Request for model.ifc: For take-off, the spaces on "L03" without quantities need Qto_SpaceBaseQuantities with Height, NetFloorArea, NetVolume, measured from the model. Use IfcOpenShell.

First a look at what the model holds.

```python
import ifcopenshell
import ifcopenshell.util.element
import ifcopenshell.util.unit

model = ifcopenshell.open("model.ifc")
print(model.schema)
for unit_type in ("LENGTHUNIT", "AREAUNIT", "VOLUMEUNIT"):
    print(unit_type, ifcopenshell.util.unit.calculate_unit_scale(model, unit_type))
storey = next(s for s in model.by_type("IfcBuildingStorey") if s.Name == "L03")
spaces = [e for e in ifcopenshell.util.element.get_decomposition(storey) if e.is_a("IfcSpace")]
for e in sorted(spaces, key=lambda e: e.id()):
    print(e.id(), e.is_a(), e.Name, list(ifcopenshell.util.element.get_psets(e, qtos_only=True)), sep=" | ")
```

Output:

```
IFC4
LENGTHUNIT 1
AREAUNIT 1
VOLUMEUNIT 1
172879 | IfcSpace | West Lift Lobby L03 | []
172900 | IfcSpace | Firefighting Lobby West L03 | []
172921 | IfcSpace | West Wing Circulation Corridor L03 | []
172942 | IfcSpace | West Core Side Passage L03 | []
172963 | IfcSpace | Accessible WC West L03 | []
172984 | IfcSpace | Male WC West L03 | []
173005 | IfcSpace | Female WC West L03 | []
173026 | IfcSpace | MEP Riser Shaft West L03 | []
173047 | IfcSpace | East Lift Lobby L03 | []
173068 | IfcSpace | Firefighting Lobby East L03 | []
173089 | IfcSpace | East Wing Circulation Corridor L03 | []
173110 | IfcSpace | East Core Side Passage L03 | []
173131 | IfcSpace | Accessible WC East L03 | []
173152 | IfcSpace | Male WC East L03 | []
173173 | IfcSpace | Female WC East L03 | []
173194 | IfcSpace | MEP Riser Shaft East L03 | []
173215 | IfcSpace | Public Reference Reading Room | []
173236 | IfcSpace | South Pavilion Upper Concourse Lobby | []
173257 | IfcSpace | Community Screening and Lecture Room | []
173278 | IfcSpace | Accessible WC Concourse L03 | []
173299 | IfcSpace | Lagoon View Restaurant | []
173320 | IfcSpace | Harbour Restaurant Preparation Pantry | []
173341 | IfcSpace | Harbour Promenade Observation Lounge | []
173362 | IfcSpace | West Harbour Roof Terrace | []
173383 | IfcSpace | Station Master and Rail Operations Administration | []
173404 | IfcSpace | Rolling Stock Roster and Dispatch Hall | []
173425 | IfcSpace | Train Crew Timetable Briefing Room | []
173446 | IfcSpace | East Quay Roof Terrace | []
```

```python
import ifcopenshell
import ifcopenshell.api.pset
import ifcopenshell.geom
import ifcopenshell.util.element
import ifcopenshell.util.shape
import ifcopenshell.util.unit

model = ifcopenshell.open("model.ifc")
unit_scale = ifcopenshell.util.unit.calculate_unit_scale(model)
area_scale = ifcopenshell.util.unit.calculate_unit_scale(model, "AREAUNIT")
volume_scale = ifcopenshell.util.unit.calculate_unit_scale(model, "VOLUMEUNIT")
settings = ifcopenshell.geom.settings()

storey = next(s for s in model.by_type("IfcBuildingStorey") if s.Name == "L03")
spaces = [e for e in ifcopenshell.util.element.get_decomposition(storey) if e.is_a("IfcSpace")]

for e in sorted(spaces, key=lambda e: e.id()):
    if ifcopenshell.util.element.get_psets(e, qtos_only=True, should_inherit=False):
        continue
    # Geometry comes back in metres, in the element's own axes.
    shape = ifcopenshell.geom.create_shape(settings, e)
    values = {
        "Height": ifcopenshell.util.shape.get_z(shape.geometry) / unit_scale,
        "NetFloorArea": ifcopenshell.util.shape.get_footprint_area(shape.geometry) / area_scale,
        "NetVolume": ifcopenshell.util.shape.get_volume(shape.geometry) / volume_scale,
    }
    qto = ifcopenshell.api.pset.add_qto(model, product=e, name="Qto_SpaceBaseQuantities")
    ifcopenshell.api.pset.edit_qto(model, qto=qto, properties=values)
    print(e.id(), {k: round(v, 3) for k, v in values.items()})

model.write("model_edited.ifc")
```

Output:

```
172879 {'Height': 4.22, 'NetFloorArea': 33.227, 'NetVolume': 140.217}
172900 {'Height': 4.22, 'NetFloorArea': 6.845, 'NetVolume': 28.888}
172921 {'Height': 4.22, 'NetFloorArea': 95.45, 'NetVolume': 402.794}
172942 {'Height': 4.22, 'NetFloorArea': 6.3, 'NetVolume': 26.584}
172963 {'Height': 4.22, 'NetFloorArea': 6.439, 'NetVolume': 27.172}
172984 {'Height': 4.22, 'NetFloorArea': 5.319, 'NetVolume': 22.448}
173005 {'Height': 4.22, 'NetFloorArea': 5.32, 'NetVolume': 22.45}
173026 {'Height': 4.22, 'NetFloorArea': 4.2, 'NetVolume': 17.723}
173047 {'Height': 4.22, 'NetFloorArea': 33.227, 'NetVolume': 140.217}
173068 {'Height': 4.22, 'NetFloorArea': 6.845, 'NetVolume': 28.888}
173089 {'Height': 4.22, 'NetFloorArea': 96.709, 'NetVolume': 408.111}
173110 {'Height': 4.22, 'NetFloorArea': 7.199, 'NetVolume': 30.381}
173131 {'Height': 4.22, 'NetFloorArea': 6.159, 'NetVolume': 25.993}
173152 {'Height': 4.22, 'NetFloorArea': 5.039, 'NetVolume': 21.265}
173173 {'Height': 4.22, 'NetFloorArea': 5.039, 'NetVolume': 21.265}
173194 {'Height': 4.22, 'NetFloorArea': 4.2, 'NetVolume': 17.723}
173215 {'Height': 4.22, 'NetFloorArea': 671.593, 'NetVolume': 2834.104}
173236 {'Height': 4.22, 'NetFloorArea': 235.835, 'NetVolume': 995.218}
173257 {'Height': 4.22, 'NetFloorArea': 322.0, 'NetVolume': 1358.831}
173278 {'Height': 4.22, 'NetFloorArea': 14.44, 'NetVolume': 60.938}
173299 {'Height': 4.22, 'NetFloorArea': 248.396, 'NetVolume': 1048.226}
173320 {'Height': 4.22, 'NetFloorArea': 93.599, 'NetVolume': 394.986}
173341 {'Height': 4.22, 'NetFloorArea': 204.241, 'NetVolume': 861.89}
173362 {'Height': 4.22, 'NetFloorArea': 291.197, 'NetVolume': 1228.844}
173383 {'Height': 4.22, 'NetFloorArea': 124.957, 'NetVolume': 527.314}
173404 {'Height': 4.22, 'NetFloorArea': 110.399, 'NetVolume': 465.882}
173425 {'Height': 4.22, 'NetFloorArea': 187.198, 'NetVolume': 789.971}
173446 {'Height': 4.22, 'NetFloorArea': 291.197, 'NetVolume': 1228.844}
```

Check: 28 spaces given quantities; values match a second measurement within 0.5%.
